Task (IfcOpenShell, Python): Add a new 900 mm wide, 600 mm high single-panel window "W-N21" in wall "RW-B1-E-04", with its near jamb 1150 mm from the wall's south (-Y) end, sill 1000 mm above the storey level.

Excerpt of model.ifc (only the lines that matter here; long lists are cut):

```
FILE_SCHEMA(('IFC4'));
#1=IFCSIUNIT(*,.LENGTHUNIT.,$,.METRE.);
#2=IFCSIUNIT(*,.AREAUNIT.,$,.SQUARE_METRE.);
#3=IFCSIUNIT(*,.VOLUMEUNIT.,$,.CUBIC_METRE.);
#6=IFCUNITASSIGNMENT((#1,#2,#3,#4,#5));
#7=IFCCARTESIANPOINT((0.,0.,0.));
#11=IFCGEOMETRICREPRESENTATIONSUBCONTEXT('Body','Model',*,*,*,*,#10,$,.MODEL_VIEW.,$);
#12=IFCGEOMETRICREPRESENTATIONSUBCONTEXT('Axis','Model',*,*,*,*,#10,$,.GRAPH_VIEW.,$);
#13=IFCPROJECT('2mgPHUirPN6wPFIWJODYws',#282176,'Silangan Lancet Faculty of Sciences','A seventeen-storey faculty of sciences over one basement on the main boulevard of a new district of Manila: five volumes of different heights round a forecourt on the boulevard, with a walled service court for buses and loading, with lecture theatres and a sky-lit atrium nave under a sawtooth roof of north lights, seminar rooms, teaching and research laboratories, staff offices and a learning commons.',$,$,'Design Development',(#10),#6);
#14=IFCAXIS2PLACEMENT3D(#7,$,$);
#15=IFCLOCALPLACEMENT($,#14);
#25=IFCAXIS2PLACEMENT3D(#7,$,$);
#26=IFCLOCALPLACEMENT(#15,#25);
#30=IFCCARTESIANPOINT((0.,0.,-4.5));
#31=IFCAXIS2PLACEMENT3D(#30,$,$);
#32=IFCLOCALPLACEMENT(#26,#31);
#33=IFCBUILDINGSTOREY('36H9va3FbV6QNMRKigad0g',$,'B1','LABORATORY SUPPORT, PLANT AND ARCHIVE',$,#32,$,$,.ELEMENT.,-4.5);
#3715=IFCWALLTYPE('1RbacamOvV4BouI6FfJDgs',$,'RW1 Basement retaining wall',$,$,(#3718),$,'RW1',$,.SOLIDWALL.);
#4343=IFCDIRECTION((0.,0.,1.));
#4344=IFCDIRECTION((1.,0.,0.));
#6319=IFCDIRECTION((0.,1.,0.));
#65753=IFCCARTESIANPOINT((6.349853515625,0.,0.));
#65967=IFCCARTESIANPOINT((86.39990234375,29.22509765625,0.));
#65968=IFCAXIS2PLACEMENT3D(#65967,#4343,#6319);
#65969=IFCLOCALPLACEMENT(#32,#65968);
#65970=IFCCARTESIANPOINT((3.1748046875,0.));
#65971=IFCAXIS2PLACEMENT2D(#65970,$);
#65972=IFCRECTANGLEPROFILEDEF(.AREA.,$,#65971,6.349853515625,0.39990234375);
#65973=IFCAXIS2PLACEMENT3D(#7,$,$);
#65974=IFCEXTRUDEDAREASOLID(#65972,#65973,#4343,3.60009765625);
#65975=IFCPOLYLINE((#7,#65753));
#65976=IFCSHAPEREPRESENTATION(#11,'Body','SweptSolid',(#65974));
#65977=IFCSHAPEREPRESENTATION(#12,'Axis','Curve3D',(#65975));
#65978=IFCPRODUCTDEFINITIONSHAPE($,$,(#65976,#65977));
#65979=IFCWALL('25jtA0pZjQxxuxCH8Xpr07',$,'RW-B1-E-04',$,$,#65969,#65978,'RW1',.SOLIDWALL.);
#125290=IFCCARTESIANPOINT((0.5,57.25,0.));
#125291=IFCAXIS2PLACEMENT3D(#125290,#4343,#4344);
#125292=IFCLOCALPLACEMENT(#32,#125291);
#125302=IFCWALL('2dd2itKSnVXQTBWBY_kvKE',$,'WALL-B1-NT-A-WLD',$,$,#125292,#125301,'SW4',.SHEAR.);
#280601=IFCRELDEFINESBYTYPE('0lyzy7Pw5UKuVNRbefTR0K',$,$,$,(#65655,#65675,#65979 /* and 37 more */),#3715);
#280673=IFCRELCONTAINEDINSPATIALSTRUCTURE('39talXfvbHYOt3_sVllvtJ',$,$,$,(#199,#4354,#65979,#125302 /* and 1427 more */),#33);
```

```python
import numpy as np
import ifcopenshell
import ifcopenshell.api.feature
import ifcopenshell.api.geometry
import ifcopenshell.api.root
import ifcopenshell.api.spatial
import ifcopenshell.geom
import ifcopenshell.util.element
import ifcopenshell.util.placement
import ifcopenshell.util.representation
import ifcopenshell.util.shape
import ifcopenshell.util.unit

model = ifcopenshell.open("model.ifc")
unit_scale = ifcopenshell.util.unit.calculate_unit_scale(model)
settings = ifcopenshell.geom.settings()


def volume(element):
    """Net volume in cubic metres, openings subtracted."""
    shape = ifcopenshell.geom.create_shape(settings, element)
    return ifcopenshell.util.shape.get_volume(shape.geometry)


wall = model.by_guid("25jtA0pZjQxxuxCH8Xpr07")
storey = ifcopenshell.util.element.get_container(wall, ifc_class="IfcBuildingStorey")
context = ifcopenshell.util.representation.get_context(model, "Model", "Body", "MODEL_VIEW")
before = volume(wall)

width, height, from_end, sill = 0.9, 0.6, 1.15, 1  # metres

# The wall runs along its own X axis, and the end named is its -X end.
wall_shape = ifcopenshell.geom.create_shape(settings, wall)
x, y, z = ifcopenshell.util.shape.get_vertices(wall_shape.geometry).T
start = x.min() + from_end
face, thickness = float(y.min()), float(y.max() - y.min())
wall_matrix = ifcopenshell.util.placement.get_local_placement(wall.ObjectPlacement)
level = ifcopenshell.util.placement.get_local_placement(storey.ObjectPlacement)[2, 3]


def in_wall(x, y):
    """Placement at x, y metres in the wall's axes, at sill height."""
    matrix = wall_matrix.copy()
    matrix[:, 3] = wall_matrix @ np.array([x / unit_scale, y / unit_scale, 0.0, 1.0])
    matrix[2, 3] = level + sill / unit_scale
    return matrix


# Opening: a box that overshoots both wall faces by 50 mm.
opening = ifcopenshell.api.root.create_entity(model, ifc_class="IfcOpeningElement", predefined_type="OPENING")
box = ifcopenshell.api.geometry.add_wall_representation(
    model, context=context, length=width, height=height, thickness=thickness + 0.1
)
ifcopenshell.api.geometry.assign_representation(model, product=opening, representation=box)
ifcopenshell.api.geometry.edit_object_placement(model, product=opening, matrix=in_wall(start, face - 0.05), is_si=False)
ifcopenshell.api.feature.add_feature(model, feature=opening, element=wall)

window = ifcopenshell.api.root.create_entity(model, ifc_class="IfcWindow", name="W-N21", predefined_type="WINDOW")
window.OverallWidth, window.OverallHeight = width / unit_scale, height / unit_scale
window.PartitioningType = "SINGLE_PANEL"
body = ifcopenshell.api.geometry.add_window_representation(
    model,
    context=context,
    overall_width=window.OverallWidth,
    overall_height=window.OverallHeight,
    partition_type="SINGLE_PANEL",
)
ifcopenshell.api.geometry.assign_representation(model, product=window, representation=body)
ifcopenshell.api.spatial.assign_container(model, products=[window], relating_structure=storey)
ifcopenshell.api.feature.add_filling(model, opening=opening, element=window)

# Centre the window in the wall's thickness.
ifcopenshell.api.geometry.edit_object_placement(model, product=window, matrix=in_wall(start, face), is_si=False)
window_shape = ifcopenshell.geom.create_shape(settings, window)
depth = ifcopenshell.util.shape.get_vertices(window_shape.geometry)[:, 1]
offset = face + thickness / 2 - (depth.min() + depth.max()) / 2
ifcopenshell.api.geometry.edit_object_placement(model, product=window, matrix=in_wall(start, offset), is_si=False)

after = volume(wall)

print(f"wall volume {before:.3f} -> {after:.3f} m3")

model.write("model_updated.ifc")
```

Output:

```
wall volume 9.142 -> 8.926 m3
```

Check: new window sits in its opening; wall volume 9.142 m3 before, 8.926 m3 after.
